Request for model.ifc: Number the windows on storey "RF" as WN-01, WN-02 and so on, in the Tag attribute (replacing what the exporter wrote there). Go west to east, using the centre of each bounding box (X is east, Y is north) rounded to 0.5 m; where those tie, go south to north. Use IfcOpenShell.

First a look at what the model holds.

```python
import ifcopenshell
import ifcopenshell.util.element
import ifcopenshell.util.placement

model = ifcopenshell.open("model.ifc")
print(model.schema)
storey = next(s for s in model.by_type("IfcBuildingStorey") if s.Name == "RF")
windows = [e for e in ifcopenshell.util.element.get_decomposition(storey) if e.is_a("IfcWindow")]
for e in sorted(windows, key=lambda e: e.id()):
    origin = ifcopenshell.util.placement.get_local_placement(e.ObjectPlacement)[:3, 3]
    print(e.id(), e.Tag, e.Name, origin.round(2) + 0.0, sep=" | ")
```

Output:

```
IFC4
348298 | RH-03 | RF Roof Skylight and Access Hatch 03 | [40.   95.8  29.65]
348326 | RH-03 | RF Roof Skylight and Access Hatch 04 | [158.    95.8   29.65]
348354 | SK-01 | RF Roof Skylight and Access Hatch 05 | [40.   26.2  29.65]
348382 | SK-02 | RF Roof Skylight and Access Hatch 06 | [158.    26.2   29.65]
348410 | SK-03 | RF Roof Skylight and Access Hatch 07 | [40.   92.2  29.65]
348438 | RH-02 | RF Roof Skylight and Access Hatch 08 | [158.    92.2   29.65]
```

```python
import ifcopenshell
import ifcopenshell.geom
import ifcopenshell.util.element
import ifcopenshell.util.shape

model = ifcopenshell.open("model.ifc")
settings = ifcopenshell.geom.settings()
settings.set("use-world-coords", True)


def centre(element):
    shape = ifcopenshell.geom.create_shape(settings, element)
    return ifcopenshell.util.shape.get_bbox_centroid(shape.geometry)


storey = next(s for s in model.by_type("IfcBuildingStorey") if s.Name == "RF")
windows = [e for e in ifcopenshell.util.element.get_decomposition(storey) if e.is_a("IfcWindow")]

# Insertion points can sit at a corner or the storey origin, so sort by the geometry (in metres).
centres = {e: centre(e) for e in windows}
windows.sort(key=lambda e: (round(centres[e][0] / 0.5), centres[e][1]))

for i, e in enumerate(windows, start=1):
    number = f"WN-{i:02d}"
    e.Tag = number
    print(e.id(), number)

model.write("model_updated.ifc")
```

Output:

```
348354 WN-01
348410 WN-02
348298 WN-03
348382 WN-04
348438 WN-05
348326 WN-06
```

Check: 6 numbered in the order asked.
